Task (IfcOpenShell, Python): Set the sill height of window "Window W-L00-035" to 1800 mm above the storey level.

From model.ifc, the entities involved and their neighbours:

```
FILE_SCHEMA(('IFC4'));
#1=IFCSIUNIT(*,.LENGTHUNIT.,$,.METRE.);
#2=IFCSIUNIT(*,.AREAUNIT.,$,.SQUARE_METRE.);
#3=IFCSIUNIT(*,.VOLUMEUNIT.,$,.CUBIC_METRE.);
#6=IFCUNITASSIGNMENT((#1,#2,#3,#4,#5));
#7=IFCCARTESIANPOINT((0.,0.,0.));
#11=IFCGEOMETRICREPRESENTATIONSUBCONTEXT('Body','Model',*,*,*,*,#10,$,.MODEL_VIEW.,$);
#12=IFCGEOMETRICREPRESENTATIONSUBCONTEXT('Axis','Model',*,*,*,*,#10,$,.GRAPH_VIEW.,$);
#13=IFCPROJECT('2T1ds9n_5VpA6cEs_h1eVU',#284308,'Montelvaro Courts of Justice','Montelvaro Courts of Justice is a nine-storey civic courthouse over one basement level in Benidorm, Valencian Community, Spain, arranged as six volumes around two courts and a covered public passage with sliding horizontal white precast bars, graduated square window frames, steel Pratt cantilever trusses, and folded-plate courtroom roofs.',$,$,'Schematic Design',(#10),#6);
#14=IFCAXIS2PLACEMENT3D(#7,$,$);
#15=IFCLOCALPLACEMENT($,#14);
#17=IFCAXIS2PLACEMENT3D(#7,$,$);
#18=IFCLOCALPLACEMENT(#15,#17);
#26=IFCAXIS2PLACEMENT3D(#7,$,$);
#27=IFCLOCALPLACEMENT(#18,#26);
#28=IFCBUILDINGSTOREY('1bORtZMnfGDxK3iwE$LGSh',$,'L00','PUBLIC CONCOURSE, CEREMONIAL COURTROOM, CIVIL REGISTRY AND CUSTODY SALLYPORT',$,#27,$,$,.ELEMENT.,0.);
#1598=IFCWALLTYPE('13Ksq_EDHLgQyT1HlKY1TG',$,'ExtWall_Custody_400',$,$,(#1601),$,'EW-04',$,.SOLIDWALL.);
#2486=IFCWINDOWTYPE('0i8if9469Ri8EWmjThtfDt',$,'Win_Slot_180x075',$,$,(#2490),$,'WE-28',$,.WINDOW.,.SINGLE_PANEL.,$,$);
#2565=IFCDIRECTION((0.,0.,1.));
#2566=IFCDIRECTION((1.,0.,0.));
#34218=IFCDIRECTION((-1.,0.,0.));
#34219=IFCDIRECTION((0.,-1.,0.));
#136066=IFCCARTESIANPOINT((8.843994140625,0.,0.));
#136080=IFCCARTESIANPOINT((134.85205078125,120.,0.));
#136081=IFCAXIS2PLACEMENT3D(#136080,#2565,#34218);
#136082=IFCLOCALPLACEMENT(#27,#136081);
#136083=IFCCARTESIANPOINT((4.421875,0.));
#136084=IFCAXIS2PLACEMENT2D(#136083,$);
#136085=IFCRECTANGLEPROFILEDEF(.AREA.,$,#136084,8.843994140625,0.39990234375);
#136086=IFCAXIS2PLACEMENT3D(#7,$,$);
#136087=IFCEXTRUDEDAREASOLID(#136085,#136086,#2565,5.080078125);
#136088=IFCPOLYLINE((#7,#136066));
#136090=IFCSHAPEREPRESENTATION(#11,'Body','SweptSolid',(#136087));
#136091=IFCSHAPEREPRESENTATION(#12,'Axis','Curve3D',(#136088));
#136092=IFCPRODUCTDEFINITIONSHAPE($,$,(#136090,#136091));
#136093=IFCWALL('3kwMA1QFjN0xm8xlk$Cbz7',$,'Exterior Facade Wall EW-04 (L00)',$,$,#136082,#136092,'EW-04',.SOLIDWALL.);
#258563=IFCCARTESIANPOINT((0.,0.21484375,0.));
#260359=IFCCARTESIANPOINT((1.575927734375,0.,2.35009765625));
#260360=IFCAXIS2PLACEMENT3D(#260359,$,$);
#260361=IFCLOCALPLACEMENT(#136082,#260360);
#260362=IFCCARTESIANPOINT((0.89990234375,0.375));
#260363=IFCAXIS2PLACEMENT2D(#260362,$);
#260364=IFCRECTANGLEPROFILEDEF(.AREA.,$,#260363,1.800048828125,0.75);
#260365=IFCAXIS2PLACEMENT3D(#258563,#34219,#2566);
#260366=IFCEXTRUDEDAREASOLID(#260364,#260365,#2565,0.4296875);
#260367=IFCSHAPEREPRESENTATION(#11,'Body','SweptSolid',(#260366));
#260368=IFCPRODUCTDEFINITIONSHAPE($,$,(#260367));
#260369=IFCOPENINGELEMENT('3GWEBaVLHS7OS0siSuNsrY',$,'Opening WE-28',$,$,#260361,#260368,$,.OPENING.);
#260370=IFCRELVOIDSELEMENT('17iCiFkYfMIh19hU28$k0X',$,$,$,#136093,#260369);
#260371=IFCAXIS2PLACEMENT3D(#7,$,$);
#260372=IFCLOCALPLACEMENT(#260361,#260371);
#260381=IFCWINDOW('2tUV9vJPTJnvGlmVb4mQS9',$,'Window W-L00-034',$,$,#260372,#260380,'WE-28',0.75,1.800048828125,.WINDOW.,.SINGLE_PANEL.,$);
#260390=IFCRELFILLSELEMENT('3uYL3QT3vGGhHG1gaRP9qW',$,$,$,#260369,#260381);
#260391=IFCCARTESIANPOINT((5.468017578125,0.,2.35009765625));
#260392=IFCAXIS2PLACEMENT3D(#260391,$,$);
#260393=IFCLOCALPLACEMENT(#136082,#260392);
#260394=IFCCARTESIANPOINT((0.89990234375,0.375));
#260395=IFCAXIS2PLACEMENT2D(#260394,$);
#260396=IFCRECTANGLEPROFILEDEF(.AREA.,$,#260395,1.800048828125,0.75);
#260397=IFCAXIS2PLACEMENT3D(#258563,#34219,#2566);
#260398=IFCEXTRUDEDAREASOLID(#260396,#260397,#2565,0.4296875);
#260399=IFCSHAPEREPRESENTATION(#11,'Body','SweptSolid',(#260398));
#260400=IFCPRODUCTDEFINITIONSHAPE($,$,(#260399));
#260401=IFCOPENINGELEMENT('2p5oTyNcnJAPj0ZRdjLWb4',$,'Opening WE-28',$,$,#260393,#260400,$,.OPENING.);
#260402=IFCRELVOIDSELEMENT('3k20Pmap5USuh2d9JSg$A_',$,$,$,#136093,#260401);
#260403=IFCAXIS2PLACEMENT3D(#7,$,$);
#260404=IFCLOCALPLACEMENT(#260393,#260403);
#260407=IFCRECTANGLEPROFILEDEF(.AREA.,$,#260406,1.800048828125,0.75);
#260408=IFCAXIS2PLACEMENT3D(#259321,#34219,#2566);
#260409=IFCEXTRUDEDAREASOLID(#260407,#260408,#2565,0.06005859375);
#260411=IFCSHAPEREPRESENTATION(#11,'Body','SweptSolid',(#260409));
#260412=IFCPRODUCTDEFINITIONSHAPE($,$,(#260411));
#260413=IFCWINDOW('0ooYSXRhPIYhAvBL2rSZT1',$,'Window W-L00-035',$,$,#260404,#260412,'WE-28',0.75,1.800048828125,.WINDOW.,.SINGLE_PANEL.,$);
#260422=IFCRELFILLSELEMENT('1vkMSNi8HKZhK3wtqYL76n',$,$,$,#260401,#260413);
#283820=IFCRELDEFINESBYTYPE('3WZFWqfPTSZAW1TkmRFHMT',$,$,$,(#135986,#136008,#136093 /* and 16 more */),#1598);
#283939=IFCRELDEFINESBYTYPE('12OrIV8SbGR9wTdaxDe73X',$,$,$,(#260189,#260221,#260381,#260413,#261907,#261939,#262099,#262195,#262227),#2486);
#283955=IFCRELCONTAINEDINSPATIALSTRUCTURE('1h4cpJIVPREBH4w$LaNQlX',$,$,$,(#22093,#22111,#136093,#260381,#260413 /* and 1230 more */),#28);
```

```python
import numpy as np
import ifcopenshell
import ifcopenshell.api.geometry
import ifcopenshell.geom
import ifcopenshell.util.element
import ifcopenshell.util.placement
import ifcopenshell.util.shape
import ifcopenshell.util.unit

model = ifcopenshell.open("model.ifc")
unit_scale = ifcopenshell.util.unit.calculate_unit_scale(model)

window = model.by_id(260413)
opening = window.FillsVoids[0].RelatingOpeningElement
storey = ifcopenshell.util.element.get_container(window, ifc_class="IfcBuildingStorey")
level = ifcopenshell.util.placement.get_local_placement(storey.ObjectPlacement)[2, 3]

# The opening's origin need not be at the sill, so measure its lowest point.
shape = ifcopenshell.geom.create_shape(ifcopenshell.geom.settings(), opening)
bottom = ifcopenshell.util.shape.get_shape_bottom_elevation(shape, shape.geometry) / unit_scale
dz = level + 1.8 / unit_scale - bottom

shift = np.array([0.0, 0.0, dz])
# The window is placed relative to its opening, so it follows when the opening moves.
matrix = ifcopenshell.util.placement.get_local_placement(opening.ObjectPlacement)
matrix[:3, 3] += shift
ifcopenshell.api.geometry.edit_object_placement(
    model, product=opening, matrix=matrix, is_si=False, should_transform_children=True
)

print(f"moved by {dz * unit_scale:+.3f} m")

model.write("model_rev.ifc")
```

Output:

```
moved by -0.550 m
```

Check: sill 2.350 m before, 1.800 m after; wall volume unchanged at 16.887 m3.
